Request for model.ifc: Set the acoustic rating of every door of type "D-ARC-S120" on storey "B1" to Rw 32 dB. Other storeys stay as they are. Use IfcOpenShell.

First a look at what the model holds.

```python
import ifcopenshell
import ifcopenshell.util.element

model = ifcopenshell.open("model.ifc")
print(model.schema)
storey = next(s for s in model.by_type("IfcBuildingStorey") if s.Name == "B1")
doors = [e for e in ifcopenshell.util.element.get_decomposition(storey) if e.is_a("IfcDoor")]
seen = {}
for e in doors:
    element_type = ifcopenshell.util.element.get_type(e)
    key = (element_type.Name if element_type != e and element_type else None, ifcopenshell.util.element.get_pset(e, "Pset_DoorCommon", "AcousticRating"))
    seen[key] = seen.get(key, 0) + 1
for (name, value), count in sorted(seen.items(), key=str):
    print(count, "x", name, "|", value)
```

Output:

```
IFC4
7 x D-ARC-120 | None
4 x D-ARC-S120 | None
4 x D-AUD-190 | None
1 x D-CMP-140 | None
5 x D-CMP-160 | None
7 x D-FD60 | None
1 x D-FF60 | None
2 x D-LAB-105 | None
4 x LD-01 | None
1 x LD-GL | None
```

```python
import ifcopenshell
import ifcopenshell.api.pset
import ifcopenshell.util.element

model = ifcopenshell.open("model.ifc")

storey = next(s for s in model.by_type("IfcBuildingStorey") if s.Name == "B1")
doors = [e for e in ifcopenshell.util.element.get_decomposition(storey) if e.is_a("IfcDoor")]

count = 0
for e in doors:
    element_type = ifcopenshell.util.element.get_type(e)
    if element_type in (None, e) or element_type.Name != "D-ARC-S120":
        continue
    # add_pset returns the element's existing set when there is one.
    pset = ifcopenshell.api.pset.add_pset(model, product=e, name="Pset_DoorCommon")
    ifcopenshell.api.pset.edit_pset(model, pset=pset, properties={"AcousticRating": "Rw 32 dB"})
    count += 1

print(count, "doors updated")

model.write("model_rev.ifc")
```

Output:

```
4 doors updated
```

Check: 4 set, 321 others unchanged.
